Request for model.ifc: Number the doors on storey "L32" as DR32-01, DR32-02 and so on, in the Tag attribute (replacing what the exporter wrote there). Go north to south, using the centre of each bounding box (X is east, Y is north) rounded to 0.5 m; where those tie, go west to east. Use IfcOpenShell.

First a look at what the model holds.

```python
import ifcopenshell
import ifcopenshell.util.element
import ifcopenshell.util.placement

model = ifcopenshell.open("model.ifc")
print(model.schema)
storey = next(s for s in model.by_type("IfcBuildingStorey") if s.Name == "L32")
doors = [e for e in ifcopenshell.util.element.get_decomposition(storey) if e.is_a("IfcDoor")]
for e in sorted(doors, key=lambda e: e.id()):
    origin = ifcopenshell.util.placement.get_local_placement(e.ObjectPlacement)[:3, 3]
    print(e.id(), e.Tag, e.Name, origin.round(2) + 0.0, sep=" | ")
```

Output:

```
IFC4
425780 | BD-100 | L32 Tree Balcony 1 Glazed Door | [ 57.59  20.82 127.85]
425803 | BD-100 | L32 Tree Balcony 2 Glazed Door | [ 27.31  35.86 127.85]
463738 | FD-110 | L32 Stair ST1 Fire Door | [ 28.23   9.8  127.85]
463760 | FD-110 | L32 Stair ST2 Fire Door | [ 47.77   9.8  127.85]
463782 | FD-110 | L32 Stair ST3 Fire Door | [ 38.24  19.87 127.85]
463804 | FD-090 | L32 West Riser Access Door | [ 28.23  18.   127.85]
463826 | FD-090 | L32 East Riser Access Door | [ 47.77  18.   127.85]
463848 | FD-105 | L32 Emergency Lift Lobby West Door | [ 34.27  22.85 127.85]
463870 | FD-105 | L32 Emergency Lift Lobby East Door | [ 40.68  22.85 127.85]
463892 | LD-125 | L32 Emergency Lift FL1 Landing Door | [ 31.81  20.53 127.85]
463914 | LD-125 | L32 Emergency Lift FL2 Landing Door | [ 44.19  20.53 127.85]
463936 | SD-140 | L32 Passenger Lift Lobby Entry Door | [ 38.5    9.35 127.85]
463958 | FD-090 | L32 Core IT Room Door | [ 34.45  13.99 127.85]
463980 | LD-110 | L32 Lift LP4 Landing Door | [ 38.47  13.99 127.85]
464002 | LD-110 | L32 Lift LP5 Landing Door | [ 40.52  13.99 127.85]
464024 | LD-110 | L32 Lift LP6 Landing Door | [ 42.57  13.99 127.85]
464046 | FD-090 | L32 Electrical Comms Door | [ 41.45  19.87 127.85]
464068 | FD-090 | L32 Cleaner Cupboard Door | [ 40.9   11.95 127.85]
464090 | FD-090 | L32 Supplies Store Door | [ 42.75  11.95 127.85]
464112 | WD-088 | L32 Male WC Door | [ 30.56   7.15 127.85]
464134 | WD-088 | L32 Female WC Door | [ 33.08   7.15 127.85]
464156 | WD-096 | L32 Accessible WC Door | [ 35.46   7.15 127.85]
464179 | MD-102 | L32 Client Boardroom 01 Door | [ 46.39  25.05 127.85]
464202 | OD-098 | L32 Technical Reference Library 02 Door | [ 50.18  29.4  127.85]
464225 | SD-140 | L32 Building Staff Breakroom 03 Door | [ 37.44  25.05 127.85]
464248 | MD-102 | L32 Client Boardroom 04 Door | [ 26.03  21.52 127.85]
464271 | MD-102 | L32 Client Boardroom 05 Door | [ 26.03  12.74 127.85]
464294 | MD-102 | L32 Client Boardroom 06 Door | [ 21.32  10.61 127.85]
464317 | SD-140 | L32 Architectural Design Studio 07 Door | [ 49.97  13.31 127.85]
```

```python
import ifcopenshell
import ifcopenshell.geom
import ifcopenshell.util.element
import ifcopenshell.util.shape

model = ifcopenshell.open("model.ifc")
settings = ifcopenshell.geom.settings()
settings.set("use-world-coords", True)


def centre(element):
    shape = ifcopenshell.geom.create_shape(settings, element)
    return ifcopenshell.util.shape.get_bbox_centroid(shape.geometry)


storey = next(s for s in model.by_type("IfcBuildingStorey") if s.Name == "L32")
doors = [e for e in ifcopenshell.util.element.get_decomposition(storey) if e.is_a("IfcDoor")]

# Insertion points can sit at a corner or the storey origin, so sort by the geometry (in metres).
centres = {e: centre(e) for e in doors}
doors.sort(key=lambda e: (-round(centres[e][1] / 0.5), centres[e][0]))

for i, e in enumerate(doors, start=1):
    number = f"DR32-{i:02d}"
    e.Tag = number
    print(e.id(), number)

model.write("model_edited.ifc")
```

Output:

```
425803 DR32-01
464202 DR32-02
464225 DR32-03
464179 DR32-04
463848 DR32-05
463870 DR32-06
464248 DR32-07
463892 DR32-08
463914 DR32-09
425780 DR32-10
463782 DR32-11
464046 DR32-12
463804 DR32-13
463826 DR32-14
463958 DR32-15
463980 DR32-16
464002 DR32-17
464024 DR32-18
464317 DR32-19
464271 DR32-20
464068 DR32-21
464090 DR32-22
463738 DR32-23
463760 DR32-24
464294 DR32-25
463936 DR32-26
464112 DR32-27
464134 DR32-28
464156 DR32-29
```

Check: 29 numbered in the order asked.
